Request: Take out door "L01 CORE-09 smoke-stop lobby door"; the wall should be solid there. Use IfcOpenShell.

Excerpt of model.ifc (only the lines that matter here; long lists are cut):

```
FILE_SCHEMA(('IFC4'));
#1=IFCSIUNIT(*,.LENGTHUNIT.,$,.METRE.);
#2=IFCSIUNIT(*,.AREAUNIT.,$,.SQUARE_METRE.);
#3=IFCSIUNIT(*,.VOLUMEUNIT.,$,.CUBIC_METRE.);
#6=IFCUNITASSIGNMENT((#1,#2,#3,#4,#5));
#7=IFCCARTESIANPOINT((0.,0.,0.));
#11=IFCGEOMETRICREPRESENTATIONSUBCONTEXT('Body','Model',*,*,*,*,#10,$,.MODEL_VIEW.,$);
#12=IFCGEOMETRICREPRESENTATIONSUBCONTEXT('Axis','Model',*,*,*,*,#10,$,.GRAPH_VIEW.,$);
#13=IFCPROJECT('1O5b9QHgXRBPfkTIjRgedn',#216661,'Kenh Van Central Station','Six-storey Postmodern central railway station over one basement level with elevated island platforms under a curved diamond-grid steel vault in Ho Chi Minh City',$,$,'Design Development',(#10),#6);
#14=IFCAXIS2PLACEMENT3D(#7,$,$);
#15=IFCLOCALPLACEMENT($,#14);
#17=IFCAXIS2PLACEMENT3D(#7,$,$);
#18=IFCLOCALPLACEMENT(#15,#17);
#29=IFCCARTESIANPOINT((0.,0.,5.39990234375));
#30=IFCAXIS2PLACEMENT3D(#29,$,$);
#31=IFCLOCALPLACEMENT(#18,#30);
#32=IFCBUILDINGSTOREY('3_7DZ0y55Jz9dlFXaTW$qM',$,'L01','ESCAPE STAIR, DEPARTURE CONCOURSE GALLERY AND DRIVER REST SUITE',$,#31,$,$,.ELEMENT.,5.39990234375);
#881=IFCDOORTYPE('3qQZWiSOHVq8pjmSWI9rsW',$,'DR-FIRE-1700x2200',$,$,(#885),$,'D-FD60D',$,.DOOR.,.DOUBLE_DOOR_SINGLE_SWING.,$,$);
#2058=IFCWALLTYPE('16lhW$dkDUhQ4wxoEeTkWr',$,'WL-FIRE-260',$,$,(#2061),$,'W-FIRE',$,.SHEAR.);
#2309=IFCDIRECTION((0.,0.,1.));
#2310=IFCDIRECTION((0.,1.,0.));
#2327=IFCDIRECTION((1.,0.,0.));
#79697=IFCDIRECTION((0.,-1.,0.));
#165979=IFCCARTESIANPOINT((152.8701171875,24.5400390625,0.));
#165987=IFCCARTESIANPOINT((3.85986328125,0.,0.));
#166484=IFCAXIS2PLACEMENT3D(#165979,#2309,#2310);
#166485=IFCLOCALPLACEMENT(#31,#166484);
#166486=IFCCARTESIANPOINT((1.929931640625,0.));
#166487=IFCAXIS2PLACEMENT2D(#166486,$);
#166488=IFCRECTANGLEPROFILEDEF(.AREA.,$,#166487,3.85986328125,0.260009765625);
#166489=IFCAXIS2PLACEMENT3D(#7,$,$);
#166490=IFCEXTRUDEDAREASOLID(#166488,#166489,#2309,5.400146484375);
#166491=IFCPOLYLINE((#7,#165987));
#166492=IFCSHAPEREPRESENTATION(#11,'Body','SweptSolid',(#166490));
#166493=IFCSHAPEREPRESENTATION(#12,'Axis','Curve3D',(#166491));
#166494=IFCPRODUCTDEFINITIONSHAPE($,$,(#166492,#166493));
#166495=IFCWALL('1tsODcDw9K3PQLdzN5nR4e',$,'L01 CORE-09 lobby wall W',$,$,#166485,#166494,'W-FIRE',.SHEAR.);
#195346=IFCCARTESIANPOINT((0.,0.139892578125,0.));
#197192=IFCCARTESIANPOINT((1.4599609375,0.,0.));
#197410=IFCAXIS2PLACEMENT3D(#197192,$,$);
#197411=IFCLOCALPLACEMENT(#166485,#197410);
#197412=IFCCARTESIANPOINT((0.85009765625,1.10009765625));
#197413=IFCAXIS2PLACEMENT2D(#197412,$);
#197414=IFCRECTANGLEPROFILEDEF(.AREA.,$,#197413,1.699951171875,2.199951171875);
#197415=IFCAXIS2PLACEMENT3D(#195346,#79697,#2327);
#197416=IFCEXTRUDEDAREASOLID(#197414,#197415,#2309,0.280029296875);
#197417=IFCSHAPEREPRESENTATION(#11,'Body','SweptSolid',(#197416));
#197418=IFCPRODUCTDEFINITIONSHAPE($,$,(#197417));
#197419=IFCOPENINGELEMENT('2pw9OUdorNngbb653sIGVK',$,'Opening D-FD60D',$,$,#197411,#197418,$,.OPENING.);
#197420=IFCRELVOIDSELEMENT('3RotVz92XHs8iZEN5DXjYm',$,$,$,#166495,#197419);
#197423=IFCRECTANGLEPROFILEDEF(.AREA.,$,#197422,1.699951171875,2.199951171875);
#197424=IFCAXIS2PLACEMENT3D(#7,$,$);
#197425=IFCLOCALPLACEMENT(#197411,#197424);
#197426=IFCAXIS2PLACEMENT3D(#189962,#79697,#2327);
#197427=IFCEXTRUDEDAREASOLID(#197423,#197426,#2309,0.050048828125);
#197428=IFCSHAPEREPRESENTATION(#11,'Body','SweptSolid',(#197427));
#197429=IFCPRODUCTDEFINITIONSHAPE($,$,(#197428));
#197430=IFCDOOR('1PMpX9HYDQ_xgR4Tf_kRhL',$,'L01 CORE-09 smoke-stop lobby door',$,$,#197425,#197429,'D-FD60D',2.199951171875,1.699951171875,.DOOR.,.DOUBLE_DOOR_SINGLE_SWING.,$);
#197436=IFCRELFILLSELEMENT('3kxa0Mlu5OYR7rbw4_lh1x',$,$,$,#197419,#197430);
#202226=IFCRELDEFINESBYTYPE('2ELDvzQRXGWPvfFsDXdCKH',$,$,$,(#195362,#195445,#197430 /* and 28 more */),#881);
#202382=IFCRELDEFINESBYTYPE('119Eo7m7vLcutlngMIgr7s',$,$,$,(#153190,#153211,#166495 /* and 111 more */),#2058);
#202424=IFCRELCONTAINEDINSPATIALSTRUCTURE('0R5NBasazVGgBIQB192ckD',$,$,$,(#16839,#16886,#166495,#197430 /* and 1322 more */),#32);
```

```python
import ifcopenshell
import ifcopenshell.api.feature
import ifcopenshell.api.root
import ifcopenshell.geom
import ifcopenshell.util.shape

model = ifcopenshell.open("model.ifc")
settings = ifcopenshell.geom.settings()


def volume(element):
    """Net volume in cubic metres, openings subtracted."""
    shape = ifcopenshell.geom.create_shape(settings, element)
    return ifcopenshell.util.shape.get_volume(shape.geometry)


door = model.by_guid("1PMpX9HYDQ_xgR4Tf_kRhL")
opening = door.FillsVoids[0].RelatingOpeningElement
wall = opening.VoidsElements[0].RelatingBuildingElement
before = volume(wall)

ifcopenshell.api.root.remove_product(model, product=door)
ifcopenshell.api.feature.remove_feature(model, feature=opening)

after = volume(wall)

print(f"wall volume {before:.3f} -> {after:.3f} m3")

model.write("model_edited.ifc")
```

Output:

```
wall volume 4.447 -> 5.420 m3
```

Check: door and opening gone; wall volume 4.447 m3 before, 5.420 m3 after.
